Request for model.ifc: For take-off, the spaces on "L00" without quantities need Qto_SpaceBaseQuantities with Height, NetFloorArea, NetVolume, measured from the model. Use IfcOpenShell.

First a look at what the model holds.

```python
import ifcopenshell
import ifcopenshell.util.element
import ifcopenshell.util.unit

model = ifcopenshell.open("model.ifc")
print(model.schema)
for unit_type in ("LENGTHUNIT", "AREAUNIT", "VOLUMEUNIT"):
    print(unit_type, ifcopenshell.util.unit.calculate_unit_scale(model, unit_type))
storey = next(s for s in model.by_type("IfcBuildingStorey") if s.Name == "L00")
spaces = [e for e in ifcopenshell.util.element.get_decomposition(storey) if e.is_a("IfcSpace")]
for e in sorted(spaces, key=lambda e: e.id()):
    print(e.id(), e.is_a(), e.Name, list(ifcopenshell.util.element.get_psets(e, qtos_only=True)), sep=" | ")
```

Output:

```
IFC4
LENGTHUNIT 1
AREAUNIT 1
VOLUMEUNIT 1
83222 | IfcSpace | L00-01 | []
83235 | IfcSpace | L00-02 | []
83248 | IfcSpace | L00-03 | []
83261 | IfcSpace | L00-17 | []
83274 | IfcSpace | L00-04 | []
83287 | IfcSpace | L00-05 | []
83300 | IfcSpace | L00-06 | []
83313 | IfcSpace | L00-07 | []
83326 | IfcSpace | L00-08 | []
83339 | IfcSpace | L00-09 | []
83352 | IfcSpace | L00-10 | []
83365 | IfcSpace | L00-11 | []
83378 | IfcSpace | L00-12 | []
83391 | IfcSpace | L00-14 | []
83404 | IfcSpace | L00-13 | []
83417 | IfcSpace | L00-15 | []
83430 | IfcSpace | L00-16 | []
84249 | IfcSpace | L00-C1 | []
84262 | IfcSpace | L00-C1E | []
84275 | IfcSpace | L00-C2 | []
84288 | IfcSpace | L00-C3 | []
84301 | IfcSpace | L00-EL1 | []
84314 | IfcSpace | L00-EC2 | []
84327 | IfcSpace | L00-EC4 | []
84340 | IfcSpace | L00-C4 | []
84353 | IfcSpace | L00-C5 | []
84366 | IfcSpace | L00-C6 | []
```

```python
import ifcopenshell
import ifcopenshell.api.pset
import ifcopenshell.geom
import ifcopenshell.util.element
import ifcopenshell.util.shape
import ifcopenshell.util.unit

model = ifcopenshell.open("model.ifc")
unit_scale = ifcopenshell.util.unit.calculate_unit_scale(model)
area_scale = ifcopenshell.util.unit.calculate_unit_scale(model, "AREAUNIT")
volume_scale = ifcopenshell.util.unit.calculate_unit_scale(model, "VOLUMEUNIT")
settings = ifcopenshell.geom.settings()

storey = next(s for s in model.by_type("IfcBuildingStorey") if s.Name == "L00")
spaces = [e for e in ifcopenshell.util.element.get_decomposition(storey) if e.is_a("IfcSpace")]

for e in sorted(spaces, key=lambda e: e.id()):
    if ifcopenshell.util.element.get_psets(e, qtos_only=True, should_inherit=False):
        continue
    # Geometry comes back in metres, in the element's own axes.
    shape = ifcopenshell.geom.create_shape(settings, e)
    values = {
        "Height": ifcopenshell.util.shape.get_z(shape.geometry) / unit_scale,
        "NetFloorArea": ifcopenshell.util.shape.get_footprint_area(shape.geometry) / area_scale,
        "NetVolume": ifcopenshell.util.shape.get_volume(shape.geometry) / volume_scale,
    }
    qto = ifcopenshell.api.pset.add_qto(model, product=e, name="Qto_SpaceBaseQuantities")
    ifcopenshell.api.pset.edit_qto(model, qto=qto, properties=values)
    print(e.id(), {k: round(v, 3) for k, v in values.items()})

model.write("model_v2.ifc")
```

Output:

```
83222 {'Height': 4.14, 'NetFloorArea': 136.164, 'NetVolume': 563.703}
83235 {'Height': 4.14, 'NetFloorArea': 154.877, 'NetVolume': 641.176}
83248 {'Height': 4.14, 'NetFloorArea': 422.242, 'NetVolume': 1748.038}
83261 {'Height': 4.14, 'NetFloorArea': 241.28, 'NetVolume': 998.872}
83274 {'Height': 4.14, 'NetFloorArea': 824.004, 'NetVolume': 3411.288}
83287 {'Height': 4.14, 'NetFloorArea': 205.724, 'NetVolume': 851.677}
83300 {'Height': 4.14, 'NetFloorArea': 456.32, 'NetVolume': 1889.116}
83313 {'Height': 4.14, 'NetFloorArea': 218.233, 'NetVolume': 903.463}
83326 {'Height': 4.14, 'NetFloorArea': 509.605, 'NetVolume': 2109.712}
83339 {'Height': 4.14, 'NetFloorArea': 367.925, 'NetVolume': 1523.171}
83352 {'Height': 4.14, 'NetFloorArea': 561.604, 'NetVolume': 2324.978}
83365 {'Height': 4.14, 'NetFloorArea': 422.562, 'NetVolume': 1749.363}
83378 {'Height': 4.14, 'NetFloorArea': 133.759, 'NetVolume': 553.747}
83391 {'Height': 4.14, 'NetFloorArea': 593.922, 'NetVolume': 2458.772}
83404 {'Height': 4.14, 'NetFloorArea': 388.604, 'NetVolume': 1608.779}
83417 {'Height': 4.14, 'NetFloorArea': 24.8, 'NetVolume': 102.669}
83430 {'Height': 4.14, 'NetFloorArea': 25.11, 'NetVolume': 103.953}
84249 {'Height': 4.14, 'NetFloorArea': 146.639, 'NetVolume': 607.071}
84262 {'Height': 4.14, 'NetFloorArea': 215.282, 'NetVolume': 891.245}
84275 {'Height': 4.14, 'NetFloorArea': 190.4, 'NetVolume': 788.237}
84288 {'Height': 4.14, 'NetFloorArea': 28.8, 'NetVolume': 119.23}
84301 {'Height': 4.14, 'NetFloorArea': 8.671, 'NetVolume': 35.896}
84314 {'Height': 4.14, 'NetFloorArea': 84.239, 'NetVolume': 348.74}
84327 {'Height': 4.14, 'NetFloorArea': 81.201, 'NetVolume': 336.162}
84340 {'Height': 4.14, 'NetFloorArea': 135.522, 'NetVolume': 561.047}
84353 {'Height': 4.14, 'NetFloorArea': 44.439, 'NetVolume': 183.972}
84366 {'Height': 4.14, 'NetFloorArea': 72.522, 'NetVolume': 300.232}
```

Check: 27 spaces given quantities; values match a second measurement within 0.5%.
